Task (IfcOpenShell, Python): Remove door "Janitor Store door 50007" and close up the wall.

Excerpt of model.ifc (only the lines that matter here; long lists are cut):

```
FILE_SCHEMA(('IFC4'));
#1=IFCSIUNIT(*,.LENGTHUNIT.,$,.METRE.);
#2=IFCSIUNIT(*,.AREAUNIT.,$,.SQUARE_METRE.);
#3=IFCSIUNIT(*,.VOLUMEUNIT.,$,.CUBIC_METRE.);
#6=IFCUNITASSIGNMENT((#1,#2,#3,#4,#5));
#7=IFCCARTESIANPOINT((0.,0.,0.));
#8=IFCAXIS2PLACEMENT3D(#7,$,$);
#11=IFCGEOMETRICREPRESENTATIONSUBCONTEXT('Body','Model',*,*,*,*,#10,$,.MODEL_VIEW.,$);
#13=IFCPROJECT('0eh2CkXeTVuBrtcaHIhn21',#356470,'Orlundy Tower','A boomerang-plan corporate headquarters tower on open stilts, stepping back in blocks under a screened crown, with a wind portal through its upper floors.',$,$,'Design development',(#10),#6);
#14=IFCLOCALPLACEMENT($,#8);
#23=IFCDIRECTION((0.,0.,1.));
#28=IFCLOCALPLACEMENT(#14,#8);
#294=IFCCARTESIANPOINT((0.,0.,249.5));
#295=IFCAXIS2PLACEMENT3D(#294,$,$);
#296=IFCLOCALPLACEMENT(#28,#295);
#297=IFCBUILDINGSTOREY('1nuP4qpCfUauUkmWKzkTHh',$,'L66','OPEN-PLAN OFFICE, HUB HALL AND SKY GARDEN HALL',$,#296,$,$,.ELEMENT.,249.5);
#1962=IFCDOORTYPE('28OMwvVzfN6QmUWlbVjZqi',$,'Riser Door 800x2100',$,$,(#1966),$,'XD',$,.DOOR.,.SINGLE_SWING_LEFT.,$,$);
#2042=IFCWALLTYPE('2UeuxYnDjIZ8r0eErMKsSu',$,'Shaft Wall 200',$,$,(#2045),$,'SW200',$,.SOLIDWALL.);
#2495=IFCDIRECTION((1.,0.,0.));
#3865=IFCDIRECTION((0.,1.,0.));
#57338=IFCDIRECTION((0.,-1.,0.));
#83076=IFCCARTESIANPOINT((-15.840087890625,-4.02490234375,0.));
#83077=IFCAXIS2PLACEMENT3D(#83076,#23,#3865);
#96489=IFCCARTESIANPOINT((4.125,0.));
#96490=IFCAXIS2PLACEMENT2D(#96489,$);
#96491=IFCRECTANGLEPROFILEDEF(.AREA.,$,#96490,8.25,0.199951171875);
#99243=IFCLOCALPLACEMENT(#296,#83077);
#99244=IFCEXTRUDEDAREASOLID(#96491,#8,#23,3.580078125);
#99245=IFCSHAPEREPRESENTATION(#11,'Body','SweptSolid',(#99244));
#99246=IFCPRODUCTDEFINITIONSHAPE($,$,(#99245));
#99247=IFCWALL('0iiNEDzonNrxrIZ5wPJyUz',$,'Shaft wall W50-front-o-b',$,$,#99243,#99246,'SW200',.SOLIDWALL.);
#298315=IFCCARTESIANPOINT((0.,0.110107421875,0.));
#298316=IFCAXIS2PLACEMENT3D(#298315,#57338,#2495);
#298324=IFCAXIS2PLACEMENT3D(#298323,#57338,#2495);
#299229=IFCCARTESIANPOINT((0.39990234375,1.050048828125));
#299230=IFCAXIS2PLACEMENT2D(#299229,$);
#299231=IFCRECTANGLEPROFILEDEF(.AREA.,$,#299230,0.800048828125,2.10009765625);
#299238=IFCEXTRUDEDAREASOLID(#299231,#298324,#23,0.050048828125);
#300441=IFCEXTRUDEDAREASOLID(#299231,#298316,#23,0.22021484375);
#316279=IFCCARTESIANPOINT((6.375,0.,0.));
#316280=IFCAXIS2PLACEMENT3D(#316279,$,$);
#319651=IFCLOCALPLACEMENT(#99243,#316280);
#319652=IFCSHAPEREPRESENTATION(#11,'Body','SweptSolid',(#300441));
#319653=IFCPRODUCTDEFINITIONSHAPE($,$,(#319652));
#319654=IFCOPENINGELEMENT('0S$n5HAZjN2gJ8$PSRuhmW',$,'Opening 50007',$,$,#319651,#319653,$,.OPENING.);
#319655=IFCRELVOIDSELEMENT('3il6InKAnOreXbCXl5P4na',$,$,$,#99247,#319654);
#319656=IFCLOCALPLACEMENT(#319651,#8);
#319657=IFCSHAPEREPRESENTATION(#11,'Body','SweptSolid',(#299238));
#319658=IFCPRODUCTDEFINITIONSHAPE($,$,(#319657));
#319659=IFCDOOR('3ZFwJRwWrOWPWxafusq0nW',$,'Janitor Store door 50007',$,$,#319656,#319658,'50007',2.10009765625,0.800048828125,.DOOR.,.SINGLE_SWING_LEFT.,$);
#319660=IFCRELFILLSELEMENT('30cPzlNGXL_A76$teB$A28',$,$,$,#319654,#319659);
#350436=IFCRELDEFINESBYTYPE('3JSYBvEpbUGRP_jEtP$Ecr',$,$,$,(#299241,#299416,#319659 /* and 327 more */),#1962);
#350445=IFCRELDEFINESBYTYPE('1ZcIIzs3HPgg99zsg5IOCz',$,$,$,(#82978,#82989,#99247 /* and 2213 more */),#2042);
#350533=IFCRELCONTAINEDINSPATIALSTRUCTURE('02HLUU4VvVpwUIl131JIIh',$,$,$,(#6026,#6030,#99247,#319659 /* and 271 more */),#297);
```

```python
import ifcopenshell
import ifcopenshell.api.feature
import ifcopenshell.api.root
import ifcopenshell.geom
import ifcopenshell.util.shape

model = ifcopenshell.open("model.ifc")
settings = ifcopenshell.geom.settings()


def volume(element):
    """Net volume in cubic metres, openings subtracted."""
    shape = ifcopenshell.geom.create_shape(settings, element)
    return ifcopenshell.util.shape.get_volume(shape.geometry)


door = model.by_guid("3ZFwJRwWrOWPWxafusq0nW")
opening = door.FillsVoids[0].RelatingOpeningElement
wall = opening.VoidsElements[0].RelatingBuildingElement
before = volume(wall)

ifcopenshell.api.root.remove_product(model, product=door)
ifcopenshell.api.feature.remove_feature(model, feature=opening)

after = volume(wall)

print(f"wall volume {before:.3f} -> {after:.3f} m3")

model.write("model_edited.ifc")
```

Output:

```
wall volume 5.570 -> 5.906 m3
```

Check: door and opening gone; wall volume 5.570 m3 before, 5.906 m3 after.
